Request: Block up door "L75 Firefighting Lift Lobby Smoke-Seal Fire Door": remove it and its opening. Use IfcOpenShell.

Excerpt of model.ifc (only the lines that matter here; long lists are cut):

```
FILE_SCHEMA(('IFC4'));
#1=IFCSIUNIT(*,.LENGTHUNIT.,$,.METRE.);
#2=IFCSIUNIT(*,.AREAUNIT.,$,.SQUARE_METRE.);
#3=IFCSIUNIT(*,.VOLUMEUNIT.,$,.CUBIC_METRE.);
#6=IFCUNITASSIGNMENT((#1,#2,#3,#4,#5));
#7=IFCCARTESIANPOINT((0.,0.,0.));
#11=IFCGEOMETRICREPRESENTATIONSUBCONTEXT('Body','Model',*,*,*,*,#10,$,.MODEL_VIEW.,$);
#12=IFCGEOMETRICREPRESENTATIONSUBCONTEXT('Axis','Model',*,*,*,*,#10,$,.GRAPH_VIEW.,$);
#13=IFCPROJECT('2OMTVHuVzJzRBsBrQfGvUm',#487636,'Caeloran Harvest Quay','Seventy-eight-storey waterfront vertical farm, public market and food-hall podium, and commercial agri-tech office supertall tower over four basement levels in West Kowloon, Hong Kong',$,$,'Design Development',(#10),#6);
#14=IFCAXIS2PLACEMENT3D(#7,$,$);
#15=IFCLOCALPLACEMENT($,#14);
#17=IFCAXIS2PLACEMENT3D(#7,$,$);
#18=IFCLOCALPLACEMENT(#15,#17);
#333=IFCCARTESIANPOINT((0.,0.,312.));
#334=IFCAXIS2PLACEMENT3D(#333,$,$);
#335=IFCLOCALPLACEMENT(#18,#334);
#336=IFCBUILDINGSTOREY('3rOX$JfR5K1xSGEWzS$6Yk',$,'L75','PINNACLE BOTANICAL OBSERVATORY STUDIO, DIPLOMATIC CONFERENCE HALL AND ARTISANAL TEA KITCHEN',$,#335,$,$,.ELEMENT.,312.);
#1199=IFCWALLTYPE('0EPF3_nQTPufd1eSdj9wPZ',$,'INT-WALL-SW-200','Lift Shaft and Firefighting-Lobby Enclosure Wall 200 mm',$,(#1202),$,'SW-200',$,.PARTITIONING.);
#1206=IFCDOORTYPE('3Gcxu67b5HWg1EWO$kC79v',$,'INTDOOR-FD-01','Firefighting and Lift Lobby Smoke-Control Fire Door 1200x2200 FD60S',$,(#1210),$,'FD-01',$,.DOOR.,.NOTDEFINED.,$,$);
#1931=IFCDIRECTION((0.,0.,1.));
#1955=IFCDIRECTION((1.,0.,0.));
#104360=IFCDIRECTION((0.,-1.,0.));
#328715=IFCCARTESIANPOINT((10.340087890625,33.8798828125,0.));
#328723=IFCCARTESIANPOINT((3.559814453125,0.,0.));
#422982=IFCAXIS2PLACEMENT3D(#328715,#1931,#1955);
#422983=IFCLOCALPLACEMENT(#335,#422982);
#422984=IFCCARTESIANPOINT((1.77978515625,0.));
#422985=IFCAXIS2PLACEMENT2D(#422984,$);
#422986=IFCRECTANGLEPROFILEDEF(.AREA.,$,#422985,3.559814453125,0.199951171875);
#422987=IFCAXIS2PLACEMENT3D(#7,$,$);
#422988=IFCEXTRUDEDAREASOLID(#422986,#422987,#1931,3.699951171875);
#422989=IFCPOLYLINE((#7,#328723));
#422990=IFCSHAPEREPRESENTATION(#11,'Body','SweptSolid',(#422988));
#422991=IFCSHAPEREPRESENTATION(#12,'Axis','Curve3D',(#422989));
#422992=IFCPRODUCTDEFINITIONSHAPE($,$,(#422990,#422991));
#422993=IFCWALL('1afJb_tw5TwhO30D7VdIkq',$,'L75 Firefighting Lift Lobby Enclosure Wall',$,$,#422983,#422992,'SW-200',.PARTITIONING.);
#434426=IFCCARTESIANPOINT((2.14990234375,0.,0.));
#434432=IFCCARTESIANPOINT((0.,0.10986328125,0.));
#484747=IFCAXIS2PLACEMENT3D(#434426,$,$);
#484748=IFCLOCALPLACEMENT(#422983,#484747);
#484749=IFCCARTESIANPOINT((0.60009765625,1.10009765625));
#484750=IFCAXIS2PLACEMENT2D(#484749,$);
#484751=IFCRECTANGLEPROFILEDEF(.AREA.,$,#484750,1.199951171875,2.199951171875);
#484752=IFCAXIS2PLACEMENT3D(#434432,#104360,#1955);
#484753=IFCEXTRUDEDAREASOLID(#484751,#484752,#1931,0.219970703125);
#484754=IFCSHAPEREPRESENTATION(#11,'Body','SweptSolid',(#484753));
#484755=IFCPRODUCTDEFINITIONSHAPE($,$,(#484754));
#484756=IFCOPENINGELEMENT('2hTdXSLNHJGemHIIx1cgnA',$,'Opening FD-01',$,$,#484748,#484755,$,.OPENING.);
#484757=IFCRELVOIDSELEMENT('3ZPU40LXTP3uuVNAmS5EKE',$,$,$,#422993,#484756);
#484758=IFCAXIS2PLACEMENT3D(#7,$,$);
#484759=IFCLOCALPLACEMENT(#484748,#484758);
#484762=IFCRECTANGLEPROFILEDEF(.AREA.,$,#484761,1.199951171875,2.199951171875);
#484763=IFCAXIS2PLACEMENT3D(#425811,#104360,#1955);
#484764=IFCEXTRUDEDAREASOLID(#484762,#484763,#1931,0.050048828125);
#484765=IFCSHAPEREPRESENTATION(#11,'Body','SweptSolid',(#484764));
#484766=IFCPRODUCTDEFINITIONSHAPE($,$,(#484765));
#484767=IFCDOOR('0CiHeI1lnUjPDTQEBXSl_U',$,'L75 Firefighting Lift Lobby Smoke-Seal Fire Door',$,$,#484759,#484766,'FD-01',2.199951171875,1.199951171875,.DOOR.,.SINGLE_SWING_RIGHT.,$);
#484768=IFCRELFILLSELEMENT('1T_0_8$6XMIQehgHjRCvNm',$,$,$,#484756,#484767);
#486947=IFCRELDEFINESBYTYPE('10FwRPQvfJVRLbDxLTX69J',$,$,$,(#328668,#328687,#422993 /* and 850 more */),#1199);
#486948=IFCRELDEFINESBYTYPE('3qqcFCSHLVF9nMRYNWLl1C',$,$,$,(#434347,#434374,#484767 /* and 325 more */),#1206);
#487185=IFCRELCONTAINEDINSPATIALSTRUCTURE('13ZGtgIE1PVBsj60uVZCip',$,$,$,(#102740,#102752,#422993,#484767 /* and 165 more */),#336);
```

```python
import ifcopenshell
import ifcopenshell.api.feature
import ifcopenshell.api.root
import ifcopenshell.geom
import ifcopenshell.util.shape

model = ifcopenshell.open("model.ifc")
settings = ifcopenshell.geom.settings()


def volume(element):
    """Net volume in cubic metres, openings subtracted."""
    shape = ifcopenshell.geom.create_shape(settings, element)
    return ifcopenshell.util.shape.get_volume(shape.geometry)


door = model.by_id(484767)
opening = door.FillsVoids[0].RelatingOpeningElement
wall = opening.VoidsElements[0].RelatingBuildingElement
before = volume(wall)

ifcopenshell.api.root.remove_product(model, product=door)
ifcopenshell.api.feature.remove_feature(model, feature=opening)

after = volume(wall)

print(f"wall volume {before:.3f} -> {after:.3f} m3")

model.write("model_edited.ifc")
```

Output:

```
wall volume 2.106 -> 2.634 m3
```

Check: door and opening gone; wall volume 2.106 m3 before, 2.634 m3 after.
